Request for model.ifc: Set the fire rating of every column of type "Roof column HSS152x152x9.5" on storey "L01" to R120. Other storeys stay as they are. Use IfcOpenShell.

First a look at what the model holds.

```python
import ifcopenshell
import ifcopenshell.util.element

model = ifcopenshell.open("model.ifc")
print(model.schema)
storey = next(s for s in model.by_type("IfcBuildingStorey") if s.Name == "L01")
columns = [e for e in ifcopenshell.util.element.get_decomposition(storey) if e.is_a("IfcColumn")]
seen = {}
for e in columns:
    element_type = ifcopenshell.util.element.get_type(e)
    key = (element_type.Name if element_type != e and element_type else None, ifcopenshell.util.element.get_pset(e, "Pset_ColumnCommon", "FireRating"))
    seen[key] = seen.get(key, 0) + 1
for (name, value), count in sorted(seen.items(), key=str):
    print(count, "x", name, "|", value)
```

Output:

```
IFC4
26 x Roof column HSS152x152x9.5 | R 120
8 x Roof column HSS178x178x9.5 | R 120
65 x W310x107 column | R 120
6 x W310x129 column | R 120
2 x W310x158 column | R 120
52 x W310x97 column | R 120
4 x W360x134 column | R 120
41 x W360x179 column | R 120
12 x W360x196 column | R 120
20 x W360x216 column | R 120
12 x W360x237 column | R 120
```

```python
import ifcopenshell
import ifcopenshell.api.pset
import ifcopenshell.util.element

model = ifcopenshell.open("model.ifc")

storey = next(s for s in model.by_type("IfcBuildingStorey") if s.Name == "L01")
columns = [e for e in ifcopenshell.util.element.get_decomposition(storey) if e.is_a("IfcColumn")]

count = 0
for e in columns:
    element_type = ifcopenshell.util.element.get_type(e)
    if element_type in (None, e) or element_type.Name != "Roof column HSS152x152x9.5":
        continue
    # add_pset returns the element's existing set when there is one.
    pset = ifcopenshell.api.pset.add_pset(model, product=e, name="Pset_ColumnCommon")
    ifcopenshell.api.pset.edit_pset(model, pset=pset, properties={"FireRating": "R120"})
    count += 1

print(count, "columns updated")

model.write("model_updated.ifc")
```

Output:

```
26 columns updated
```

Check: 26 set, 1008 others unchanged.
